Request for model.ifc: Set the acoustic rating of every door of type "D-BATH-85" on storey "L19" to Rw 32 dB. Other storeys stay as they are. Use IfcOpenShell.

First a look at what the model holds.

```python
import ifcopenshell
import ifcopenshell.util.element

model = ifcopenshell.open("model.ifc")
print(model.schema)
storey = next(s for s in model.by_type("IfcBuildingStorey") if s.Name == "L19")
doors = [e for e in ifcopenshell.util.element.get_decomposition(storey) if e.is_a("IfcDoor")]
seen = {}
for e in doors:
    element_type = ifcopenshell.util.element.get_type(e)
    key = (element_type.Name if element_type != e and element_type else None, ifcopenshell.util.element.get_pset(e, "Pset_DoorCommon", "AcousticRating"))
    seen[key] = seen.get(key, 0) + 1
for (name, value), count in sorted(seen.items(), key=str):
    print(count, "x", name, "|", value)
```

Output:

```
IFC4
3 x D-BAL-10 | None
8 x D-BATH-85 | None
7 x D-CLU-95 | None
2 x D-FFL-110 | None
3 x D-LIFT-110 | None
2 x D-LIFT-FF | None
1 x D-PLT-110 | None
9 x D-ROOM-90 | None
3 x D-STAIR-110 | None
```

```python
import ifcopenshell
import ifcopenshell.api.pset
import ifcopenshell.util.element

model = ifcopenshell.open("model.ifc")

storey = next(s for s in model.by_type("IfcBuildingStorey") if s.Name == "L19")
doors = [e for e in ifcopenshell.util.element.get_decomposition(storey) if e.is_a("IfcDoor")]

count = 0
for e in doors:
    element_type = ifcopenshell.util.element.get_type(e)
    if element_type in (None, e) or element_type.Name != "D-BATH-85":
        continue
    found = ifcopenshell.util.element.get_pset(e, "Pset_DoorCommon", should_inherit=False)
    if found:
        pset = model.by_id(found["id"])
        if len(ifcopenshell.util.element.get_elements_by_pset(pset)) > 1:
            pset = ifcopenshell.api.pset.unshare_pset(model, products=[e], pset=pset)[0]
    else:
        pset = ifcopenshell.api.pset.add_pset(model, product=e, name="Pset_DoorCommon")
    ifcopenshell.api.pset.edit_pset(model, pset=pset, properties={"AcousticRating": "Rw 32 dB"})
    count += 1

print(count, "doors updated")

model.write("model_rev.ifc")
```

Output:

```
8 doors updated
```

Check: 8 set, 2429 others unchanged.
